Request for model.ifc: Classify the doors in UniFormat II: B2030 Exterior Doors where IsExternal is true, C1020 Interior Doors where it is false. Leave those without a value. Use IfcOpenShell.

First a look at what the model holds.

```python
import ifcopenshell
import ifcopenshell.util.element

model = ifcopenshell.open("model.ifc")
print(model.schema)
print("classifications:", [c.Name for c in model.by_type("IfcClassification")])
values = [ifcopenshell.util.element.get_pset(e, "Pset_DoorCommon", "IsExternal") for e in model.by_type("IfcDoor")]
for value in (True, False, None):
    print("IsExternal", value, values.count(value))
```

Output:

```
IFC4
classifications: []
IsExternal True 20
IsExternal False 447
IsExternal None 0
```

```python
import ifcopenshell
import ifcopenshell.api.classification
import ifcopenshell.util.element

model = ifcopenshell.open("model.ifc")

system = ifcopenshell.api.classification.add_classification(model, classification="UniFormat II")

doors = model.by_type("IfcDoor")
external = {e: ifcopenshell.util.element.get_pset(e, "Pset_DoorCommon", "IsExternal") for e in doors}
for flag, code, name in ((True, "B2030", "Exterior Doors"), (False, "C1020", "Interior Doors")):
    products = [e for e in doors if external[e] is flag]
    ifcopenshell.api.classification.add_reference(
        model, products=products, classification=system, identification=code, name=name
    )
    print(code, len(products))

model.write("model_v2.ifc")
```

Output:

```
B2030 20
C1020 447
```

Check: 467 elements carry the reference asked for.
